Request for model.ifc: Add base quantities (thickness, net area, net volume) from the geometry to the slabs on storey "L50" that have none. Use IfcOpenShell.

First a look at what the model holds.

```python
import ifcopenshell
import ifcopenshell.util.element
import ifcopenshell.util.unit

model = ifcopenshell.open("model.ifc")
print(model.schema)
for unit_type in ("LENGTHUNIT", "AREAUNIT", "VOLUMEUNIT"):
    print(unit_type, ifcopenshell.util.unit.calculate_unit_scale(model, unit_type))
storey = next(s for s in model.by_type("IfcBuildingStorey") if s.Name == "L50")
slabs = [e for e in ifcopenshell.util.element.get_decomposition(storey) if e.is_a("IfcSlab")]
for e in sorted(slabs, key=lambda e: e.id()):
    print(e.id(), e.is_a(), e.Name, list(ifcopenshell.util.element.get_psets(e, qtos_only=True)), sep=" | ")
```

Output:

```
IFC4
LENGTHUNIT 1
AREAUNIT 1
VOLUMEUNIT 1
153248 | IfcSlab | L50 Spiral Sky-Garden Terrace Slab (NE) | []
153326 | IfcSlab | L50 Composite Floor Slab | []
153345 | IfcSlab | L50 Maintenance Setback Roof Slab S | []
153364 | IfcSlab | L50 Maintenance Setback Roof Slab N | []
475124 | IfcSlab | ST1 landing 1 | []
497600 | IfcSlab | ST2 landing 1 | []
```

```python
import ifcopenshell
import ifcopenshell.api.pset
import ifcopenshell.geom
import ifcopenshell.util.element
import ifcopenshell.util.shape
import ifcopenshell.util.unit

model = ifcopenshell.open("model.ifc")
unit_scale = ifcopenshell.util.unit.calculate_unit_scale(model)
area_scale = ifcopenshell.util.unit.calculate_unit_scale(model, "AREAUNIT")
volume_scale = ifcopenshell.util.unit.calculate_unit_scale(model, "VOLUMEUNIT")
settings = ifcopenshell.geom.settings()

storey = next(s for s in model.by_type("IfcBuildingStorey") if s.Name == "L50")
slabs = [e for e in ifcopenshell.util.element.get_decomposition(storey) if e.is_a("IfcSlab")]

for e in sorted(slabs, key=lambda e: e.id()):
    if ifcopenshell.util.element.get_psets(e, qtos_only=True, should_inherit=False):
        continue
    # Geometry comes back in metres, in the element's own axes.
    shape = ifcopenshell.geom.create_shape(settings, e)
    values = {
        "Width": ifcopenshell.util.shape.get_z(shape.geometry) / unit_scale,
        "NetArea": ifcopenshell.util.shape.get_footprint_area(shape.geometry) / area_scale,
        "NetVolume": ifcopenshell.util.shape.get_volume(shape.geometry) / volume_scale,
    }
    qto = ifcopenshell.api.pset.add_qto(model, product=e, name="Qto_SlabBaseQuantities")
    ifcopenshell.api.pset.edit_qto(model, qto=qto, properties=values)
    print(e.id(), {k: round(v, 3) for k, v in values.items()})

model.write("model_rev.ifc")
```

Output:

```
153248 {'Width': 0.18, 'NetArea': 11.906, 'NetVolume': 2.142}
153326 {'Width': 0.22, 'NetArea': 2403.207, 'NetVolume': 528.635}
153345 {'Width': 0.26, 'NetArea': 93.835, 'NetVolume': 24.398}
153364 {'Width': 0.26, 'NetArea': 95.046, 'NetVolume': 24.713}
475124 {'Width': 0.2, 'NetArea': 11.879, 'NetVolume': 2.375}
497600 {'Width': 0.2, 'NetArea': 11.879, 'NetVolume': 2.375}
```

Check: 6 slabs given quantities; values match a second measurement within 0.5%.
